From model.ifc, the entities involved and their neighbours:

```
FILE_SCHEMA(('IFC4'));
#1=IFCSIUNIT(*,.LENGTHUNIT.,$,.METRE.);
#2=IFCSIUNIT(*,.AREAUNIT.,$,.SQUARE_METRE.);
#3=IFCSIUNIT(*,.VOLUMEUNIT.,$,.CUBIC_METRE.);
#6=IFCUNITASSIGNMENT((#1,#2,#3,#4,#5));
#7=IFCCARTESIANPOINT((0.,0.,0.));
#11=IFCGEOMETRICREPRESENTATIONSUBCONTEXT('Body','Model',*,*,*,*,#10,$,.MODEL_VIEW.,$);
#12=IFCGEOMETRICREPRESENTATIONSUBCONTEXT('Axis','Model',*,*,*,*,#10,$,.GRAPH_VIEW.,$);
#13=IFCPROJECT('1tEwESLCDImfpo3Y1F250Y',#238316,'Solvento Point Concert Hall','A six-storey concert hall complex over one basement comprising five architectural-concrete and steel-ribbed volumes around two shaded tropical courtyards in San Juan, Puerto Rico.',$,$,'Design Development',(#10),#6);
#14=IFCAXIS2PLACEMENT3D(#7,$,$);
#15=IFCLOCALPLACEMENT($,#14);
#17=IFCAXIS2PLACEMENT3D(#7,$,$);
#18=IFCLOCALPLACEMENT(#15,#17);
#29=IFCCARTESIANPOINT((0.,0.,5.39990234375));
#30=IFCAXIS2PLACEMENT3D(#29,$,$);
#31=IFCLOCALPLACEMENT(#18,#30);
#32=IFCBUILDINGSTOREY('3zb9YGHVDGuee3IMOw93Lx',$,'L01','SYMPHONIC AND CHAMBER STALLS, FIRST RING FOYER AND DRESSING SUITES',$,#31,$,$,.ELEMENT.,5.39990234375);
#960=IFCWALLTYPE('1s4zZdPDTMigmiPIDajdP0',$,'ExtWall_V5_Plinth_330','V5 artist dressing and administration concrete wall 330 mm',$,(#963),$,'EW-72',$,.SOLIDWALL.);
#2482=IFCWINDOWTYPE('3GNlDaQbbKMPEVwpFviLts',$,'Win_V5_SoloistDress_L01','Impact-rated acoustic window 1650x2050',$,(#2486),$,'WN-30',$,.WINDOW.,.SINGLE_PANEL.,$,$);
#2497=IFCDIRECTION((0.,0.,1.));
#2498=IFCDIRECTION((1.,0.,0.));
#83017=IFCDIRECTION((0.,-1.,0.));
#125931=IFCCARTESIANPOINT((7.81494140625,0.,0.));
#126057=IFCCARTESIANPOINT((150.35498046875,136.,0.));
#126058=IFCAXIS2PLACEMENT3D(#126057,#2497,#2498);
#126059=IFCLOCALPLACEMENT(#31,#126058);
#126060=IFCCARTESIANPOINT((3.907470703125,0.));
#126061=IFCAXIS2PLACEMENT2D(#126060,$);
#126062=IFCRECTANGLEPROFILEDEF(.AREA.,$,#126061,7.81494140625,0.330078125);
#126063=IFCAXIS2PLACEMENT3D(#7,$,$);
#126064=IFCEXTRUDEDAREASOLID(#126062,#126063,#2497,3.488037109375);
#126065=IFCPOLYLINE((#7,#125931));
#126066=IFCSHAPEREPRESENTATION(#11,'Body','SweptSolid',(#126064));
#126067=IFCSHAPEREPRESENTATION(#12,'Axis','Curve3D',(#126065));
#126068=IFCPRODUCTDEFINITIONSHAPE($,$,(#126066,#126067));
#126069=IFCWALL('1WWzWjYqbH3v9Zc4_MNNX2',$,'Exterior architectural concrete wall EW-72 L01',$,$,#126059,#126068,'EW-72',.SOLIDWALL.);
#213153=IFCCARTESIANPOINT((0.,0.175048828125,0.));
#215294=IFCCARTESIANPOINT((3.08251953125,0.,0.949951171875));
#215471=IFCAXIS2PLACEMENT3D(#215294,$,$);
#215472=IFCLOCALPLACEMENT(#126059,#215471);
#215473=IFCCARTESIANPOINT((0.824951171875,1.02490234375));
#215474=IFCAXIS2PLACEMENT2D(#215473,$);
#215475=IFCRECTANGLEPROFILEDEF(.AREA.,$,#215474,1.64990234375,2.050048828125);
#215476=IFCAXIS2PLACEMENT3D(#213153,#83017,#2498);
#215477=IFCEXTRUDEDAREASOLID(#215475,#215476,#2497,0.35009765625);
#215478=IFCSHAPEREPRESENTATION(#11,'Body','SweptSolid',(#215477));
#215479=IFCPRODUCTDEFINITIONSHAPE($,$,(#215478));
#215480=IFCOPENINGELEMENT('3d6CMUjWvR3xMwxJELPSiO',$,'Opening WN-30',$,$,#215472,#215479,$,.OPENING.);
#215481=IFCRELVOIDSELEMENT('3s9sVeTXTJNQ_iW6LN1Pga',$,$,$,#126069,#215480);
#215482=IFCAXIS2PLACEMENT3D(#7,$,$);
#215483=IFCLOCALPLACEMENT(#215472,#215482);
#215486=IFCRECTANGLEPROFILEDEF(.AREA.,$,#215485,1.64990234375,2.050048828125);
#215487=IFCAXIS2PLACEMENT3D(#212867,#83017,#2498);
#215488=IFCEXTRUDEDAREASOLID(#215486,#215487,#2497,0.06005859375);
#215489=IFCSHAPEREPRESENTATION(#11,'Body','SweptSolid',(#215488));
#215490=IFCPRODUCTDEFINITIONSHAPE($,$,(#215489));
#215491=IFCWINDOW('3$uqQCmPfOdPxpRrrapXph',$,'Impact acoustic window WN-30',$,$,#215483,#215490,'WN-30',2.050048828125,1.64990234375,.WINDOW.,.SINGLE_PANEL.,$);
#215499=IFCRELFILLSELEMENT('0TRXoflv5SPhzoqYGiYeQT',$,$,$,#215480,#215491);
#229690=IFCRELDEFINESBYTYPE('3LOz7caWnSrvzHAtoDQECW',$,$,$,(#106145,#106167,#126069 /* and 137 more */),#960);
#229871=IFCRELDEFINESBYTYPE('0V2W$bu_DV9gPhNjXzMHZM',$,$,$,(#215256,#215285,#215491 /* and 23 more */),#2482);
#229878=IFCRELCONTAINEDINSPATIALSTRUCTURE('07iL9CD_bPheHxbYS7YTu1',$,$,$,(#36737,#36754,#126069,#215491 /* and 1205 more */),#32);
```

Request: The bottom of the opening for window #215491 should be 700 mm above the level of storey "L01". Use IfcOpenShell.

```python
import numpy as np
import ifcopenshell
import ifcopenshell.api.geometry
import ifcopenshell.geom
import ifcopenshell.util.element
import ifcopenshell.util.placement
import ifcopenshell.util.shape
import ifcopenshell.util.unit

model = ifcopenshell.open("model.ifc")
unit_scale = ifcopenshell.util.unit.calculate_unit_scale(model)

window = model.by_guid("3$uqQCmPfOdPxpRrrapXph")
opening = window.FillsVoids[0].RelatingOpeningElement
storey = ifcopenshell.util.element.get_container(window, ifc_class="IfcBuildingStorey")
level = ifcopenshell.util.placement.get_local_placement(storey.ObjectPlacement)[2, 3]

# The opening's origin need not be at the sill, so measure its lowest point.
shape = ifcopenshell.geom.create_shape(ifcopenshell.geom.settings(), opening)
bottom = ifcopenshell.util.shape.get_shape_bottom_elevation(shape, shape.geometry) / unit_scale
dz = level + 0.7 / unit_scale - bottom

shift = np.array([0.0, 0.0, dz])
# The window is placed relative to its opening, so it follows when the opening moves.
matrix = ifcopenshell.util.placement.get_local_placement(opening.ObjectPlacement)
matrix[:3, 3] += shift
ifcopenshell.api.geometry.edit_object_placement(
    model, product=opening, matrix=matrix, is_si=False, should_transform_children=True
)

print(f"moved by {dz * unit_scale:+.3f} m")

model.write("model_edited.ifc")
```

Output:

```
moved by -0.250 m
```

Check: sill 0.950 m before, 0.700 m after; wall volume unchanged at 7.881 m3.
